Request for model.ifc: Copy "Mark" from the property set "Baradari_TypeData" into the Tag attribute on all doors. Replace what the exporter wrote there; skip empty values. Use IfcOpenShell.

First a look at what the model holds.

```python
import ifcopenshell
import ifcopenshell.util.element

model = ifcopenshell.open("model.ifc")
print(model.schema)
doors = model.by_type("IfcDoor")
print(len(doors), "doors")
for e in doors[:8]:
    source = ifcopenshell.util.element.get_pset(e, "Baradari_TypeData", "Mark")
    target = e.Tag
    print(e.id(), repr(source), repr(target), sep=" | ")
```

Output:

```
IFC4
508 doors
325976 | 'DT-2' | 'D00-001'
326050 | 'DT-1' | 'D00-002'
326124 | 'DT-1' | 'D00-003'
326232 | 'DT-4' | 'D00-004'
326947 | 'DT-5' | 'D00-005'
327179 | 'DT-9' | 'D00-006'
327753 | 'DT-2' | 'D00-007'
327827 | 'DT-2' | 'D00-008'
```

```python
import ifcopenshell
import ifcopenshell.util.element

model = ifcopenshell.open("model.ifc")

count = 0
for e in model.by_type("IfcDoor"):
    value = ifcopenshell.util.element.get_pset(e, "Baradari_TypeData", "Mark")
    current = e.Tag
    if not value or not value.strip() or current == value:
        continue
    e.Tag = value
    count += 1

print(count, "doors updated")

model.write("model_updated.ifc")
```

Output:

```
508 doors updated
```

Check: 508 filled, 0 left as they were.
